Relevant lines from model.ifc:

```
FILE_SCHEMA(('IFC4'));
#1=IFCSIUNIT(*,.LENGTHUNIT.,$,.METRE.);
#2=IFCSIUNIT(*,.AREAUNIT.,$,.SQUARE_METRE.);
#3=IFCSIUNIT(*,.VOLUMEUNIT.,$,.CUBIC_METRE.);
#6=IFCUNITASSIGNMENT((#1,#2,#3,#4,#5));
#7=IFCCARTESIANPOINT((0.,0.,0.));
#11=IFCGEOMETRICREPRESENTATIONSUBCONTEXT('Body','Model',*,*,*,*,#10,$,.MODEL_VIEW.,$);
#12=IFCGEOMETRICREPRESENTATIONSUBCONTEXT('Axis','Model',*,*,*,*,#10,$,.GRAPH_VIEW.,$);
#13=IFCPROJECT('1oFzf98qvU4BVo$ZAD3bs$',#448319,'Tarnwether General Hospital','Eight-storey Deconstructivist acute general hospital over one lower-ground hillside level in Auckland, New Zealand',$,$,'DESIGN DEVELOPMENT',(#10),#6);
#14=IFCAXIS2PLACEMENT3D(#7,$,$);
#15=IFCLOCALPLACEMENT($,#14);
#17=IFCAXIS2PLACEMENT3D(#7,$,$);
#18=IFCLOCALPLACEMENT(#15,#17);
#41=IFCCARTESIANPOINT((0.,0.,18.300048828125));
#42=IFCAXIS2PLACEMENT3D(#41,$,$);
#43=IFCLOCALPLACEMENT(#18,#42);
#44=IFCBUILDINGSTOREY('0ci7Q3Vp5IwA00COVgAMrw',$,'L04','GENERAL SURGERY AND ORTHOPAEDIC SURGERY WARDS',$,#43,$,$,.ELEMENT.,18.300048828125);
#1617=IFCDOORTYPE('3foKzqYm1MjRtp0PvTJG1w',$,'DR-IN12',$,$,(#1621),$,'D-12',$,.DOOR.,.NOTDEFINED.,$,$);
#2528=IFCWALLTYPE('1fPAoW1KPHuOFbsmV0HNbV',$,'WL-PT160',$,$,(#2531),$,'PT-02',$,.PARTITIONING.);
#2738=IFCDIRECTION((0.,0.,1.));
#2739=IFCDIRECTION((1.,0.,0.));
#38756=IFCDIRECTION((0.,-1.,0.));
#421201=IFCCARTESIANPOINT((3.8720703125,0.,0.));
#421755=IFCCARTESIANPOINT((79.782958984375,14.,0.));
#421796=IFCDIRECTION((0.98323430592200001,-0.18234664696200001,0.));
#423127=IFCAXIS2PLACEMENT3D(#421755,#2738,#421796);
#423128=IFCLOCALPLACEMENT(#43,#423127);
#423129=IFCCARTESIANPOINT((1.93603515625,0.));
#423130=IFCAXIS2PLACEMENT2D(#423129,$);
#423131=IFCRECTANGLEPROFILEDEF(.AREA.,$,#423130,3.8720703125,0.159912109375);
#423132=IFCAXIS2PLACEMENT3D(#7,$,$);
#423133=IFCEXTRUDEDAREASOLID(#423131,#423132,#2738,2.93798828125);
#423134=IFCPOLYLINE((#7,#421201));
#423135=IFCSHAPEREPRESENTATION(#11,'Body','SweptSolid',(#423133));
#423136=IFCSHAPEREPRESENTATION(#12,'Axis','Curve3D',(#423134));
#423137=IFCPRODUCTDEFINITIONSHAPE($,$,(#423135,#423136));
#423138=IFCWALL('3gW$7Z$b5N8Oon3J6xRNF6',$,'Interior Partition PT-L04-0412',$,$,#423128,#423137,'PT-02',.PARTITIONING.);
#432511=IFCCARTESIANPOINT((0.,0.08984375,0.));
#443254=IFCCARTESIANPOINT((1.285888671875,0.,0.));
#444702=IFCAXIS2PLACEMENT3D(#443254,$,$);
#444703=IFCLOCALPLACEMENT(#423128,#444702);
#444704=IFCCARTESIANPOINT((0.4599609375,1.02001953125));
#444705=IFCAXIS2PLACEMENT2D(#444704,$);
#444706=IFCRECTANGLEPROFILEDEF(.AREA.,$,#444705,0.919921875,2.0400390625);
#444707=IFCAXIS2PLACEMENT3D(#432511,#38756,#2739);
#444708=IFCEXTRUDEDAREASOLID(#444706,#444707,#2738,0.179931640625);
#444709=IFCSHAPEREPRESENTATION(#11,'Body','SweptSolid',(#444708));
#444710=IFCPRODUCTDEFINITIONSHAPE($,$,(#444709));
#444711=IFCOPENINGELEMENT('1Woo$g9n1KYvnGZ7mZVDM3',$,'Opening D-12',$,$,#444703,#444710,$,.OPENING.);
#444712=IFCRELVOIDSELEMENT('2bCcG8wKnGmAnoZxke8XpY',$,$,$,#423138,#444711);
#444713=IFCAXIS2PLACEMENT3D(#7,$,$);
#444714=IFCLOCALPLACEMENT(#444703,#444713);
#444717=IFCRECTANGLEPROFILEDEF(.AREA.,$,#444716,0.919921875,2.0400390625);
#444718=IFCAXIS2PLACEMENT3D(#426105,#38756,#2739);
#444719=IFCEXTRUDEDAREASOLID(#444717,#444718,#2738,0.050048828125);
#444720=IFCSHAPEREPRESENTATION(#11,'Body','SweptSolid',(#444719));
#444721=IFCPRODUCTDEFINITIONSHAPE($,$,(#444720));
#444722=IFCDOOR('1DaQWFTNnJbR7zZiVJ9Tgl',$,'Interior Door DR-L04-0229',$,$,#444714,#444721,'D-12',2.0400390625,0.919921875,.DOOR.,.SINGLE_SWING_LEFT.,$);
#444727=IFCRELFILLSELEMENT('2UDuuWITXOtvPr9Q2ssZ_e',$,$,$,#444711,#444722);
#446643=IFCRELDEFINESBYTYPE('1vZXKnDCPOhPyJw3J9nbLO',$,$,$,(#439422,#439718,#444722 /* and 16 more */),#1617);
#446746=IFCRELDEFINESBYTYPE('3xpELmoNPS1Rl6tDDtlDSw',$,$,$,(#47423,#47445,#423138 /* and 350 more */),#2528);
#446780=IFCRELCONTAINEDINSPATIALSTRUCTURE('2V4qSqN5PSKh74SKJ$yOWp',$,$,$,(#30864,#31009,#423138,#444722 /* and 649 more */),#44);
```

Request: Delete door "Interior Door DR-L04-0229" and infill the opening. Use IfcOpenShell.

```python
import ifcopenshell
import ifcopenshell.api.feature
import ifcopenshell.api.root
import ifcopenshell.geom
import ifcopenshell.util.shape

model = ifcopenshell.open("model.ifc")
settings = ifcopenshell.geom.settings()


def volume(element):
    """Net volume in cubic metres, openings subtracted."""
    shape = ifcopenshell.geom.create_shape(settings, element)
    return ifcopenshell.util.shape.get_volume(shape.geometry)


door = model.by_guid("1DaQWFTNnJbR7zZiVJ9Tgl")
opening = door.FillsVoids[0].RelatingOpeningElement
wall = opening.VoidsElements[0].RelatingBuildingElement
before = volume(wall)

ifcopenshell.api.root.remove_product(model, product=door)
ifcopenshell.api.feature.remove_feature(model, feature=opening)

after = volume(wall)

print(f"wall volume {before:.3f} -> {after:.3f} m3")

model.write("model_v2.ifc")
```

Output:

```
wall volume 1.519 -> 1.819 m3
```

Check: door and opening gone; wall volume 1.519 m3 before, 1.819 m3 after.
